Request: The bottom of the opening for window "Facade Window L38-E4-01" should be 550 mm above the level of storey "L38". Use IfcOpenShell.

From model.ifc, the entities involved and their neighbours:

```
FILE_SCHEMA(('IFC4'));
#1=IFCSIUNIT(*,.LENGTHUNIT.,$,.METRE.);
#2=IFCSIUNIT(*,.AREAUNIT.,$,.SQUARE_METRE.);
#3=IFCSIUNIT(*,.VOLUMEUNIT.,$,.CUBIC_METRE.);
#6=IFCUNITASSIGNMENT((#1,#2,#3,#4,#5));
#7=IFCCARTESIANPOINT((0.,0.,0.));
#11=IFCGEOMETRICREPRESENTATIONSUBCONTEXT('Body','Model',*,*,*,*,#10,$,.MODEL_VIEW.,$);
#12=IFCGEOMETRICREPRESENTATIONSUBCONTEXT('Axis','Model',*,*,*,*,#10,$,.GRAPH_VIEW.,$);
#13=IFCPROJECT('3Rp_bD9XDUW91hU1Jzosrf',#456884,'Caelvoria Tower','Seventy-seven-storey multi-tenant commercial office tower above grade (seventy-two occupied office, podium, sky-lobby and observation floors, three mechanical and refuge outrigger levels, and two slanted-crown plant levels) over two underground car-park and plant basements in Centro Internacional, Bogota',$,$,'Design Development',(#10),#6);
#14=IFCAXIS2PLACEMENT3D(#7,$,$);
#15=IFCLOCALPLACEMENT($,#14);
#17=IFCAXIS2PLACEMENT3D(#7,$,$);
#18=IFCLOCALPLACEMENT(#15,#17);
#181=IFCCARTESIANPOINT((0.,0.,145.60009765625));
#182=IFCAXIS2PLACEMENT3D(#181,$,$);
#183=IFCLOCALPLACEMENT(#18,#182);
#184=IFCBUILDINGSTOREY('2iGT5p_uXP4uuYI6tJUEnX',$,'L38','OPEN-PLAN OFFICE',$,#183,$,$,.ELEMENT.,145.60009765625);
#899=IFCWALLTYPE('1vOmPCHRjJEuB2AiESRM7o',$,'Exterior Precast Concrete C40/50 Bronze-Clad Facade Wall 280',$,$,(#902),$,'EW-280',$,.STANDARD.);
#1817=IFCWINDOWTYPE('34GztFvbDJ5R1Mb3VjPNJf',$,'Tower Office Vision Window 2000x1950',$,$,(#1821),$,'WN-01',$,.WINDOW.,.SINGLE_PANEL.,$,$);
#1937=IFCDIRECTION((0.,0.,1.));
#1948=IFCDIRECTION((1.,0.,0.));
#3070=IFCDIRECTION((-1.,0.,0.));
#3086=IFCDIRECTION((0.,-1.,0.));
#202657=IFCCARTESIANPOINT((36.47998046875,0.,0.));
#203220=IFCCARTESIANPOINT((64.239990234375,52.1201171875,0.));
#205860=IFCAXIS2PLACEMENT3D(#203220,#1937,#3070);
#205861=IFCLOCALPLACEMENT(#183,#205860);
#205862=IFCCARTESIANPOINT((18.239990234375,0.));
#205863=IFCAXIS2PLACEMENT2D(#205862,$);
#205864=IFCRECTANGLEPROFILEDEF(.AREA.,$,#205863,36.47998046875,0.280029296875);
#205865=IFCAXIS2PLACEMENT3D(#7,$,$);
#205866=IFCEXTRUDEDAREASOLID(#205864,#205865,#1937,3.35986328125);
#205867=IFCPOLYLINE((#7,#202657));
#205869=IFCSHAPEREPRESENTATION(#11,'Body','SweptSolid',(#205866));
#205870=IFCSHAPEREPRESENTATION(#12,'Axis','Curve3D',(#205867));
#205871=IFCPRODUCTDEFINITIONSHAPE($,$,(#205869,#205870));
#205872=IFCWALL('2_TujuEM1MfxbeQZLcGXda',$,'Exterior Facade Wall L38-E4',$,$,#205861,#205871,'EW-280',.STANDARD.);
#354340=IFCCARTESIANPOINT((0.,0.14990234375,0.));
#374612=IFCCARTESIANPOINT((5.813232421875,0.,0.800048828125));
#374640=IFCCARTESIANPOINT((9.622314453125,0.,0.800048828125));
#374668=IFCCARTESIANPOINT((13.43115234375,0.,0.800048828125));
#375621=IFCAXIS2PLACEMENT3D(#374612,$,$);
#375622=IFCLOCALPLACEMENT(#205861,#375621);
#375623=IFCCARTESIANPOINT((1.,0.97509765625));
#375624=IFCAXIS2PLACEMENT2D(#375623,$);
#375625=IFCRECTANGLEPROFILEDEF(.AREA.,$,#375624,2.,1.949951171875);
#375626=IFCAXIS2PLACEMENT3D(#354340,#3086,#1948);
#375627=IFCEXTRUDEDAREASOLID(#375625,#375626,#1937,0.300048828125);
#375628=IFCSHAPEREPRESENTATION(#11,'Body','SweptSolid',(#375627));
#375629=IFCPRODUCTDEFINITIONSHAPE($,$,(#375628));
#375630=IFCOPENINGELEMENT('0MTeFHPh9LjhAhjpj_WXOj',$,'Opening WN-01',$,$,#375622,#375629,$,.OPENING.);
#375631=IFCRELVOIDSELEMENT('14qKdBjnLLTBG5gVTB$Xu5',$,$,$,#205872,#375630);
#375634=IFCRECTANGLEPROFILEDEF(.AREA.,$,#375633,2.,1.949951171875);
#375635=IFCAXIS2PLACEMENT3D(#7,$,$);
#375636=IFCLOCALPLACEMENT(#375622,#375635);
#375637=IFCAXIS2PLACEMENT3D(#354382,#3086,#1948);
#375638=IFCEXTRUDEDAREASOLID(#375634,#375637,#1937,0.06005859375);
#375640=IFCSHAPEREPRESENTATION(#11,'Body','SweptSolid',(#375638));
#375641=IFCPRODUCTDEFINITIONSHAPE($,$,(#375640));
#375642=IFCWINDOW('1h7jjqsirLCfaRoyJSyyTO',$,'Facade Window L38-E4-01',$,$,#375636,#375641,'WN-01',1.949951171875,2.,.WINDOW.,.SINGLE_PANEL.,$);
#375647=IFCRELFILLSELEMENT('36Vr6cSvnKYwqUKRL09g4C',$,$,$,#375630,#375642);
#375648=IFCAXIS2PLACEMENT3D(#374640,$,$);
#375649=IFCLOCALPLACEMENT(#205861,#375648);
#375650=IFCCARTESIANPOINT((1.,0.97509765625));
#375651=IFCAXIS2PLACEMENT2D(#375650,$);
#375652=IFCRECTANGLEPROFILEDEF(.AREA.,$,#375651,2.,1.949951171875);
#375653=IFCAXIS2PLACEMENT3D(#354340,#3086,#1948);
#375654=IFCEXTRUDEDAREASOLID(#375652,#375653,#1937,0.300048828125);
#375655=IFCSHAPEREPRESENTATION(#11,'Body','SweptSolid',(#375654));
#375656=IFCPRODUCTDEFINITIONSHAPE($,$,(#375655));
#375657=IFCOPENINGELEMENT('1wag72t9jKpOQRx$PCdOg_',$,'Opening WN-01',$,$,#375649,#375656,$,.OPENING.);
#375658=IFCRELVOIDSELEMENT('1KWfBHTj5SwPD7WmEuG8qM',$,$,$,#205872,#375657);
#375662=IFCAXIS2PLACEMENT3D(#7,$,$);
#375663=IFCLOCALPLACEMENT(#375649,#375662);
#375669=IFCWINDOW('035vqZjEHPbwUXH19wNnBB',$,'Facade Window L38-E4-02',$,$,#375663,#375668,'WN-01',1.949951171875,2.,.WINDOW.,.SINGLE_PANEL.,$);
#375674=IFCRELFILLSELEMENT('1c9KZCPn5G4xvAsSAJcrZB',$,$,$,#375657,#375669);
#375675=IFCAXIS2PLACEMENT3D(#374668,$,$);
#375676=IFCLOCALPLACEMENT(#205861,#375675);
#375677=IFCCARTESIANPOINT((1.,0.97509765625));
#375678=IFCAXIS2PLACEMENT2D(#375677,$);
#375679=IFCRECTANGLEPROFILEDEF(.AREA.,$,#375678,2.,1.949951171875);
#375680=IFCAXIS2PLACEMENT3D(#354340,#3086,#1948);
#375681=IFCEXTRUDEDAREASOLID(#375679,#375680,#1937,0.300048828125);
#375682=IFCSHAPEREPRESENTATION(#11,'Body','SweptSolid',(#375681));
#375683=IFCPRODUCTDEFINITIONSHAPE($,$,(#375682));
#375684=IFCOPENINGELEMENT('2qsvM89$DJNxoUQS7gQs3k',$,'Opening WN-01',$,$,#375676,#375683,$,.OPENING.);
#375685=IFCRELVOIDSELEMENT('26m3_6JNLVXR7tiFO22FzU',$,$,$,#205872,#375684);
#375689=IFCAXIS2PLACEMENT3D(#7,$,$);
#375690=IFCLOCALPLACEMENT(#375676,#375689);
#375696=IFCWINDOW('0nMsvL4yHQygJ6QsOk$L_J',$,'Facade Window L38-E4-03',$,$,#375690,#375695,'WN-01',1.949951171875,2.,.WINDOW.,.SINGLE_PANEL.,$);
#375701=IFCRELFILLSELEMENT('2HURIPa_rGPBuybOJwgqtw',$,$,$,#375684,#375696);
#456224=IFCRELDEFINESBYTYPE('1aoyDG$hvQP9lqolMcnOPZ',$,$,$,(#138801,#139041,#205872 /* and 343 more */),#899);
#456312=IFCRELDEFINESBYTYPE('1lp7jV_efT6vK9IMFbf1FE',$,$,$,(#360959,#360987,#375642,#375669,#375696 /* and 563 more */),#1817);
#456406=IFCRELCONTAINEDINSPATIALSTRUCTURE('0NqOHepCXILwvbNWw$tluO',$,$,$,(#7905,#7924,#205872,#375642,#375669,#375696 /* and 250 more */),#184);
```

```python
import numpy as np
import ifcopenshell
import ifcopenshell.api.geometry
import ifcopenshell.geom
import ifcopenshell.util.element
import ifcopenshell.util.placement
import ifcopenshell.util.shape
import ifcopenshell.util.unit

model = ifcopenshell.open("model.ifc")
unit_scale = ifcopenshell.util.unit.calculate_unit_scale(model)

window = model.by_guid("1h7jjqsirLCfaRoyJSyyTO")
opening = window.FillsVoids[0].RelatingOpeningElement
storey = ifcopenshell.util.element.get_container(window, ifc_class="IfcBuildingStorey")
level = ifcopenshell.util.placement.get_local_placement(storey.ObjectPlacement)[2, 3]

# The opening's origin need not be at the sill, so measure its lowest point.
shape = ifcopenshell.geom.create_shape(ifcopenshell.geom.settings(), opening)
bottom = ifcopenshell.util.shape.get_shape_bottom_elevation(shape, shape.geometry) / unit_scale
dz = level + 0.55 - bottom

shift = np.array([0.0, 0.0, dz])
# The window is placed relative to its opening, so it follows when the opening moves.
matrix = ifcopenshell.util.placement.get_local_placement(opening.ObjectPlacement)
matrix[:3, 3] += shift
ifcopenshell.api.geometry.edit_object_placement(
    model, product=opening, matrix=matrix, is_si=False, should_transform_children=True
)

print(f"moved by {dz * unit_scale:+.3f} m")

model.write("model_v2.ifc")
```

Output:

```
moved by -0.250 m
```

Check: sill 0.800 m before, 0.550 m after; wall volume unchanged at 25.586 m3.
